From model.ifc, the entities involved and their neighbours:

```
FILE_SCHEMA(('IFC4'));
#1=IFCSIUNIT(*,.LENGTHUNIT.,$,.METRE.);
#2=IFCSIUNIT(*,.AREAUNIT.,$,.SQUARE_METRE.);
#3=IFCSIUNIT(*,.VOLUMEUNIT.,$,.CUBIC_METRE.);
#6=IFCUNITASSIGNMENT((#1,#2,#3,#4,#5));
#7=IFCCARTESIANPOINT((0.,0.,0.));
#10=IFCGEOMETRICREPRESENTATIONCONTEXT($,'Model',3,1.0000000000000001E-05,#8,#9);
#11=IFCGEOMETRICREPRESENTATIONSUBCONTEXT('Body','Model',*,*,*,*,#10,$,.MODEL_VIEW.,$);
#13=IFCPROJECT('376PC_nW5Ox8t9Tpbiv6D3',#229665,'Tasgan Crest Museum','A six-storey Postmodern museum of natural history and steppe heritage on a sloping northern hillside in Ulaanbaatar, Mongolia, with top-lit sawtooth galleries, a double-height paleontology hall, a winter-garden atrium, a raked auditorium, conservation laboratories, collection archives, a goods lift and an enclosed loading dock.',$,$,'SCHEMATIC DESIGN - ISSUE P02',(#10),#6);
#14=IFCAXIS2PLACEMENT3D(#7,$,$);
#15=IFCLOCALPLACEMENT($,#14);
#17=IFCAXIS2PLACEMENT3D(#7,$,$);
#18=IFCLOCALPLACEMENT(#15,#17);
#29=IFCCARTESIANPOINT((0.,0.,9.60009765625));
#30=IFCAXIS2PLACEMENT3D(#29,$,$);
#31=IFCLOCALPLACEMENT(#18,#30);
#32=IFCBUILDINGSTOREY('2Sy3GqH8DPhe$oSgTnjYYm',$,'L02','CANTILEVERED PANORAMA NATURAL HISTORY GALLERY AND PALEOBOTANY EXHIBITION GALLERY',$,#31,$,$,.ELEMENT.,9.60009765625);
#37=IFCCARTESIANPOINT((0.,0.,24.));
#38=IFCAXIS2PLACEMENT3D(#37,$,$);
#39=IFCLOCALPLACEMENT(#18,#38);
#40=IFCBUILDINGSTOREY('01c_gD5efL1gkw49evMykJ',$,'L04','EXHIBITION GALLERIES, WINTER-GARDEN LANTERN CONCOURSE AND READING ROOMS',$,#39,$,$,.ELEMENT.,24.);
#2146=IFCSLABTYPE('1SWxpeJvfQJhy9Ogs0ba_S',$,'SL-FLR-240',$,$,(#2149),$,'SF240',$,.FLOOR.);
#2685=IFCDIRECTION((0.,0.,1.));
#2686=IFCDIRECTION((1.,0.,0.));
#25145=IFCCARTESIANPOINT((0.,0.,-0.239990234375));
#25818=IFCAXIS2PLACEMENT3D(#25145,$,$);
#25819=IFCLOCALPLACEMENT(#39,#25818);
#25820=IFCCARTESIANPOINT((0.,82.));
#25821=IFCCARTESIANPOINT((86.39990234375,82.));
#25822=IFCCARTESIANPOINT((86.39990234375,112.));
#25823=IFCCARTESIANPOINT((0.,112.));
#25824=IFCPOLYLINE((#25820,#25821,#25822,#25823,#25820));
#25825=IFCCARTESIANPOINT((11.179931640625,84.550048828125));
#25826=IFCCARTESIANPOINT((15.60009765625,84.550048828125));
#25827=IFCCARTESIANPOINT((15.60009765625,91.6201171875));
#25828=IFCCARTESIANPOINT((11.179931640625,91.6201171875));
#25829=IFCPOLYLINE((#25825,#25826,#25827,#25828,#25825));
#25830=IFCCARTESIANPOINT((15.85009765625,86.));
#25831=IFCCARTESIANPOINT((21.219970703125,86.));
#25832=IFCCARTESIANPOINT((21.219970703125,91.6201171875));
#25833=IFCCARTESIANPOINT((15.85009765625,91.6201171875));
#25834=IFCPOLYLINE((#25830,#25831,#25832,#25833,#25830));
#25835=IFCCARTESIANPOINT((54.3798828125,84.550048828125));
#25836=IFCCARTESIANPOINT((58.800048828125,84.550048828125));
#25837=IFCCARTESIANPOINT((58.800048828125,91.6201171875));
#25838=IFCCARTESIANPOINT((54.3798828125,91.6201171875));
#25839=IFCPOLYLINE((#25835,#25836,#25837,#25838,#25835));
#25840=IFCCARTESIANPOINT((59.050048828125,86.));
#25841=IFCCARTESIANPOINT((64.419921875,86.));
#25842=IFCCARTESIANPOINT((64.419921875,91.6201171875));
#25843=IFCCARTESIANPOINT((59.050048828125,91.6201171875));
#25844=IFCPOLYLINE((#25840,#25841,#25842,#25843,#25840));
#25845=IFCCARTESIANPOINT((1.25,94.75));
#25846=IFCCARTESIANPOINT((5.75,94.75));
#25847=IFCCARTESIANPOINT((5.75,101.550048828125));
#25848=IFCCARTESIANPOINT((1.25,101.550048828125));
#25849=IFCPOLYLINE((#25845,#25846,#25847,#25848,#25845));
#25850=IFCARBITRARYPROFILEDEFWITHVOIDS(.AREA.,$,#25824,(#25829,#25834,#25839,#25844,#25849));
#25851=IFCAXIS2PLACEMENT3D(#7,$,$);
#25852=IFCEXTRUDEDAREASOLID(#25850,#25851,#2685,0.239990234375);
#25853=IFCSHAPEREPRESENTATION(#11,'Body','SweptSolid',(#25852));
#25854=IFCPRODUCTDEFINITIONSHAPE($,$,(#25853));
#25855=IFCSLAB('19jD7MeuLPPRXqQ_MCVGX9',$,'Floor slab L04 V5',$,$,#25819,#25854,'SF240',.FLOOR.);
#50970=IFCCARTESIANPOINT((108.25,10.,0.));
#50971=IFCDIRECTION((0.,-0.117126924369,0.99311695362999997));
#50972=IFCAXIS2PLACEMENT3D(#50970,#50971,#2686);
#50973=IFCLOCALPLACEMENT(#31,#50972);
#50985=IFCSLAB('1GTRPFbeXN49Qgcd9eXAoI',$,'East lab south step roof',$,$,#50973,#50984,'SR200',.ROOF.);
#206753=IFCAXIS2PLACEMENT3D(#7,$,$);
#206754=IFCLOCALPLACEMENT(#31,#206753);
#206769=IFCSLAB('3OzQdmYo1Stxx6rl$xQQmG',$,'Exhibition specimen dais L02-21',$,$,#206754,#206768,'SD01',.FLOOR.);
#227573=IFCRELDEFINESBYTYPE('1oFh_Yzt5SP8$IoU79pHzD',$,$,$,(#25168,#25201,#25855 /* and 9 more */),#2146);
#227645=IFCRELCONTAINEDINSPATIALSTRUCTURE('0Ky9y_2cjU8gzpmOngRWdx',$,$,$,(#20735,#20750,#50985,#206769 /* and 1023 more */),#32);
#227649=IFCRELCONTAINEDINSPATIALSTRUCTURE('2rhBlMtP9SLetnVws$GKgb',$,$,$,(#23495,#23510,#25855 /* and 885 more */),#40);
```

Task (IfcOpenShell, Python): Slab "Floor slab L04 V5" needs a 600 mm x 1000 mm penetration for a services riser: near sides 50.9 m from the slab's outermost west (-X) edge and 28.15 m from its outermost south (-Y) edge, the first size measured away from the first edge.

```python
import numpy as np
import ifcopenshell
import ifcopenshell.api.feature
import ifcopenshell.api.geometry
import ifcopenshell.api.root
import ifcopenshell.geom
import ifcopenshell.util.placement
import ifcopenshell.util.representation
import ifcopenshell.util.shape
import ifcopenshell.util.unit

model = ifcopenshell.open("model.ifc")
unit_scale = ifcopenshell.util.unit.calculate_unit_scale(model)
settings = ifcopenshell.geom.settings()


def volume(element):
    """Net volume in cubic metres, openings subtracted."""
    shape = ifcopenshell.geom.create_shape(settings, element)
    return ifcopenshell.util.shape.get_volume(shape.geometry)


slab = model.by_guid("19jD7MeuLPPRXqQ_MCVGX9")
before = volume(slab)

# Extent in the slab's own axes, in metres. The edges named are its -X and -Y sides.
slab_shape = ifcopenshell.geom.create_shape(settings, slab)
vertices = ifcopenshell.util.shape.get_vertices(slab_shape.geometry)
x_min, y_min, bottom = vertices.min(axis=0)
top = vertices[:, 2].max()

opening = ifcopenshell.api.root.create_entity(model, ifc_class="IfcOpeningElement", name="Services riser opening", predefined_type="OPENING")
context = ifcopenshell.util.representation.get_context(model, "Model", "Body", "MODEL_VIEW")
width, depth = 0.6, 1
outline = [(0.0, 0.0), (width, 0.0), (width, depth), (0.0, depth), (0.0, 0.0)]
# Overshoot both faces by 50 mm so the cut is clean.
shape = ifcopenshell.api.geometry.add_slab_representation(
    model, context=context, depth=top - bottom + 0.1, polyline=outline
)
ifcopenshell.api.geometry.assign_representation(model, product=opening, representation=shape)

matrix = ifcopenshell.util.placement.get_local_placement(slab.ObjectPlacement)
matrix[:, 3] = matrix @ np.append(np.array([x_min + 50.9, y_min + 28.15, bottom - 0.05]) / unit_scale, 1.0)
ifcopenshell.api.geometry.edit_object_placement(model, product=opening, matrix=matrix, is_si=False)
ifcopenshell.api.feature.add_feature(model, feature=opening, element=slab)

after = volume(slab)

print(f"slab volume {before:.3f} -> {after:.3f} m3")

model.write("model_updated.ifc")
```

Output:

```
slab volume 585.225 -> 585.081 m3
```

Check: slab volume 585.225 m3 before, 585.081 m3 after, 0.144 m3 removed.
